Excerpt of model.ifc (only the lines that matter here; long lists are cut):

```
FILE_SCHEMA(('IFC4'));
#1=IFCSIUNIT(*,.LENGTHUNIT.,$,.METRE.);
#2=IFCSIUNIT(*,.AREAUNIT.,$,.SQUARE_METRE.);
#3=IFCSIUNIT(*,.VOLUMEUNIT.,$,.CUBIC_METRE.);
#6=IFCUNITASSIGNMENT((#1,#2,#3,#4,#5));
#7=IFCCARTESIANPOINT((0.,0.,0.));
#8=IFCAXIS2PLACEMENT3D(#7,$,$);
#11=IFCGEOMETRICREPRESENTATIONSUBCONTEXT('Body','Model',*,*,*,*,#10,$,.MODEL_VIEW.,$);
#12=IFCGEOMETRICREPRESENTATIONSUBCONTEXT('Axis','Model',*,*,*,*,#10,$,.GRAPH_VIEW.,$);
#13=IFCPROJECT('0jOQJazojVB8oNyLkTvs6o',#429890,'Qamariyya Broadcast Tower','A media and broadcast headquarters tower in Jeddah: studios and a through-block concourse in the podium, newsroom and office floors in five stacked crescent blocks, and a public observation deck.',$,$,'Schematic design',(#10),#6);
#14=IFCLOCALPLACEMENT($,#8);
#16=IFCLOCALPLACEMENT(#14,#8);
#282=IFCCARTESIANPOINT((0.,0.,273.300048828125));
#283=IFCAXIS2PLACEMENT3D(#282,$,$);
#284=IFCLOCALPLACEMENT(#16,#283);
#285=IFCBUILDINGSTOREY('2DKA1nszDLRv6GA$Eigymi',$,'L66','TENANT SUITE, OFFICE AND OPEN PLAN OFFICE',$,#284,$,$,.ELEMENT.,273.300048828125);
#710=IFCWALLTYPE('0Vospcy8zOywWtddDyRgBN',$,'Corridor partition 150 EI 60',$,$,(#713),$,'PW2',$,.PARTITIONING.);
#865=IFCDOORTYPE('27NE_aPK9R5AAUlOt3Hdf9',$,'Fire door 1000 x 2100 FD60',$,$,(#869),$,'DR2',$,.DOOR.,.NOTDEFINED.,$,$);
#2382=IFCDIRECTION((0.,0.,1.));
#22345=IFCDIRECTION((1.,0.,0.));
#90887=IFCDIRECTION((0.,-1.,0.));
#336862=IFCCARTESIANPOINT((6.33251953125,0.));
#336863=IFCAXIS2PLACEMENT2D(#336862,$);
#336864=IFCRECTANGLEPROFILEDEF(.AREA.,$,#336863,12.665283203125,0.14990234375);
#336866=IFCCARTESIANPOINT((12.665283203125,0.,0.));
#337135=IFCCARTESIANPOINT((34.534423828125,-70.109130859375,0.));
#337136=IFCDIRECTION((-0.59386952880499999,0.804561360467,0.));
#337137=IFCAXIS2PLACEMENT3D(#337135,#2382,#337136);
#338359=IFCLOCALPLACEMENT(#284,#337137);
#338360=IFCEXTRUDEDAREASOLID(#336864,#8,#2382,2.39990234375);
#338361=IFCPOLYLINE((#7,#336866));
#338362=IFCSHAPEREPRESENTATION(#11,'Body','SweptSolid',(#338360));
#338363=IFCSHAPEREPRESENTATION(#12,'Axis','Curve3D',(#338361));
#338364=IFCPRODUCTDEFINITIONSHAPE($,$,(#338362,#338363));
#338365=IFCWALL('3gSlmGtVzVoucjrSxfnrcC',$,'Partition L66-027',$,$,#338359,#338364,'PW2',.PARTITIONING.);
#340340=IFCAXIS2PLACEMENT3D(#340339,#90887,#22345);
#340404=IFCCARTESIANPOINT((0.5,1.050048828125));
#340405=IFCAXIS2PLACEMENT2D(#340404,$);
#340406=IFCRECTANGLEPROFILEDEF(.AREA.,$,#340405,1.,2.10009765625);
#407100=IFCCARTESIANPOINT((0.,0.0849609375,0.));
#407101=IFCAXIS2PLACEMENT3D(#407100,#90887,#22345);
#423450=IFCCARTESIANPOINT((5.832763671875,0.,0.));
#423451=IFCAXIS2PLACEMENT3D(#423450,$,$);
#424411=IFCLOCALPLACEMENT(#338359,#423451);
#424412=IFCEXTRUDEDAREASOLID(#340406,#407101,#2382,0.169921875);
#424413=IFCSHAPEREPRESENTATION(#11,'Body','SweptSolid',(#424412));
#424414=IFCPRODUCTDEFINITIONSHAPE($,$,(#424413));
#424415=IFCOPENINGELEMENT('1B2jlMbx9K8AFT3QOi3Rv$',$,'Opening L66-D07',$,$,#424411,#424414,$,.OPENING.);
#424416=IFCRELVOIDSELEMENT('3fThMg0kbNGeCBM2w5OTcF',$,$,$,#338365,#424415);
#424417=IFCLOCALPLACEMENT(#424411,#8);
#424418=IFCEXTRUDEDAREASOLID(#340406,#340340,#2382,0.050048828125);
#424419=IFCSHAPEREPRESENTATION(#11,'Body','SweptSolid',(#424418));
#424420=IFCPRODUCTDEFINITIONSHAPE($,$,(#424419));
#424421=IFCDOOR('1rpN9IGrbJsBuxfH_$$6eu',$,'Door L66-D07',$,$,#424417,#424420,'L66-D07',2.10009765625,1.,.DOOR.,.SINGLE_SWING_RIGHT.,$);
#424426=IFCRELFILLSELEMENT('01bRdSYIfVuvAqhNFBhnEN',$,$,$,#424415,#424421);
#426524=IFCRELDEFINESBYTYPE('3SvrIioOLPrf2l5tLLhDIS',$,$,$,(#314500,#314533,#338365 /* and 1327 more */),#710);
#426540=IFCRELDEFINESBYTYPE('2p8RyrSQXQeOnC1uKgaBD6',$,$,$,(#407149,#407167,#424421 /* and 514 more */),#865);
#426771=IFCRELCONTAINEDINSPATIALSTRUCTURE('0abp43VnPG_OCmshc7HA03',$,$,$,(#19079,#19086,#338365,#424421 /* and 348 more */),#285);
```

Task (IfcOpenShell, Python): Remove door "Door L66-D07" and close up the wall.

```python
import ifcopenshell
import ifcopenshell.api.feature
import ifcopenshell.api.root
import ifcopenshell.geom
import ifcopenshell.util.shape

model = ifcopenshell.open("model.ifc")
settings = ifcopenshell.geom.settings()


def volume(element):
    """Net volume in cubic metres, openings subtracted."""
    shape = ifcopenshell.geom.create_shape(settings, element)
    return ifcopenshell.util.shape.get_volume(shape.geometry)


door = model.by_id(424421)
opening = door.FillsVoids[0].RelatingOpeningElement
wall = opening.VoidsElements[0].RelatingBuildingElement
before = volume(wall)

ifcopenshell.api.root.remove_product(model, product=door)
ifcopenshell.api.feature.remove_feature(model, feature=opening)

after = volume(wall)

print(f"wall volume {before:.3f} -> {after:.3f} m3")

model.write("model-out.ifc")
```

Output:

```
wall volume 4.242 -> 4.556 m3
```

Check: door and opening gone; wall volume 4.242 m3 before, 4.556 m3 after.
